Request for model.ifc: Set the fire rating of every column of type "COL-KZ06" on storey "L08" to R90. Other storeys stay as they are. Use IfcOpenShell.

First a look at what the model holds.

```python
import ifcopenshell
import ifcopenshell.util.element

model = ifcopenshell.open("model.ifc")
print(model.schema)
storey = next(s for s in model.by_type("IfcBuildingStorey") if s.Name == "L08")
columns = [e for e in ifcopenshell.util.element.get_decomposition(storey) if e.is_a("IfcColumn")]
seen = {}
for e in columns:
    element_type = ifcopenshell.util.element.get_type(e)
    key = (element_type.Name if element_type != e and element_type else None, ifcopenshell.util.element.get_pset(e, "Pset_ColumnCommon", "FireRating"))
    seen[key] = seen.get(key, 0) + 1
for (name, value), count in sorted(seen.items(), key=str):
    print(count, "x", name, "|", value)
```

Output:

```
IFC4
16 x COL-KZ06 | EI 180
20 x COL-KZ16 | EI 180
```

```python
import ifcopenshell
import ifcopenshell.api.pset
import ifcopenshell.util.element

model = ifcopenshell.open("model.ifc")

storey = next(s for s in model.by_type("IfcBuildingStorey") if s.Name == "L08")
columns = [e for e in ifcopenshell.util.element.get_decomposition(storey) if e.is_a("IfcColumn")]

count = 0
for e in columns:
    element_type = ifcopenshell.util.element.get_type(e)
    if element_type in (None, e) or element_type.Name != "COL-KZ06":
        continue
    # add_pset returns the element's existing set when there is one.
    pset = ifcopenshell.api.pset.add_pset(model, product=e, name="Pset_ColumnCommon")
    ifcopenshell.api.pset.edit_pset(model, pset=pset, properties={"FireRating": "R90"})
    count += 1

print(count, "columns updated")

model.write("model_edited.ifc")
```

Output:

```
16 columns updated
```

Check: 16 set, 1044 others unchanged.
